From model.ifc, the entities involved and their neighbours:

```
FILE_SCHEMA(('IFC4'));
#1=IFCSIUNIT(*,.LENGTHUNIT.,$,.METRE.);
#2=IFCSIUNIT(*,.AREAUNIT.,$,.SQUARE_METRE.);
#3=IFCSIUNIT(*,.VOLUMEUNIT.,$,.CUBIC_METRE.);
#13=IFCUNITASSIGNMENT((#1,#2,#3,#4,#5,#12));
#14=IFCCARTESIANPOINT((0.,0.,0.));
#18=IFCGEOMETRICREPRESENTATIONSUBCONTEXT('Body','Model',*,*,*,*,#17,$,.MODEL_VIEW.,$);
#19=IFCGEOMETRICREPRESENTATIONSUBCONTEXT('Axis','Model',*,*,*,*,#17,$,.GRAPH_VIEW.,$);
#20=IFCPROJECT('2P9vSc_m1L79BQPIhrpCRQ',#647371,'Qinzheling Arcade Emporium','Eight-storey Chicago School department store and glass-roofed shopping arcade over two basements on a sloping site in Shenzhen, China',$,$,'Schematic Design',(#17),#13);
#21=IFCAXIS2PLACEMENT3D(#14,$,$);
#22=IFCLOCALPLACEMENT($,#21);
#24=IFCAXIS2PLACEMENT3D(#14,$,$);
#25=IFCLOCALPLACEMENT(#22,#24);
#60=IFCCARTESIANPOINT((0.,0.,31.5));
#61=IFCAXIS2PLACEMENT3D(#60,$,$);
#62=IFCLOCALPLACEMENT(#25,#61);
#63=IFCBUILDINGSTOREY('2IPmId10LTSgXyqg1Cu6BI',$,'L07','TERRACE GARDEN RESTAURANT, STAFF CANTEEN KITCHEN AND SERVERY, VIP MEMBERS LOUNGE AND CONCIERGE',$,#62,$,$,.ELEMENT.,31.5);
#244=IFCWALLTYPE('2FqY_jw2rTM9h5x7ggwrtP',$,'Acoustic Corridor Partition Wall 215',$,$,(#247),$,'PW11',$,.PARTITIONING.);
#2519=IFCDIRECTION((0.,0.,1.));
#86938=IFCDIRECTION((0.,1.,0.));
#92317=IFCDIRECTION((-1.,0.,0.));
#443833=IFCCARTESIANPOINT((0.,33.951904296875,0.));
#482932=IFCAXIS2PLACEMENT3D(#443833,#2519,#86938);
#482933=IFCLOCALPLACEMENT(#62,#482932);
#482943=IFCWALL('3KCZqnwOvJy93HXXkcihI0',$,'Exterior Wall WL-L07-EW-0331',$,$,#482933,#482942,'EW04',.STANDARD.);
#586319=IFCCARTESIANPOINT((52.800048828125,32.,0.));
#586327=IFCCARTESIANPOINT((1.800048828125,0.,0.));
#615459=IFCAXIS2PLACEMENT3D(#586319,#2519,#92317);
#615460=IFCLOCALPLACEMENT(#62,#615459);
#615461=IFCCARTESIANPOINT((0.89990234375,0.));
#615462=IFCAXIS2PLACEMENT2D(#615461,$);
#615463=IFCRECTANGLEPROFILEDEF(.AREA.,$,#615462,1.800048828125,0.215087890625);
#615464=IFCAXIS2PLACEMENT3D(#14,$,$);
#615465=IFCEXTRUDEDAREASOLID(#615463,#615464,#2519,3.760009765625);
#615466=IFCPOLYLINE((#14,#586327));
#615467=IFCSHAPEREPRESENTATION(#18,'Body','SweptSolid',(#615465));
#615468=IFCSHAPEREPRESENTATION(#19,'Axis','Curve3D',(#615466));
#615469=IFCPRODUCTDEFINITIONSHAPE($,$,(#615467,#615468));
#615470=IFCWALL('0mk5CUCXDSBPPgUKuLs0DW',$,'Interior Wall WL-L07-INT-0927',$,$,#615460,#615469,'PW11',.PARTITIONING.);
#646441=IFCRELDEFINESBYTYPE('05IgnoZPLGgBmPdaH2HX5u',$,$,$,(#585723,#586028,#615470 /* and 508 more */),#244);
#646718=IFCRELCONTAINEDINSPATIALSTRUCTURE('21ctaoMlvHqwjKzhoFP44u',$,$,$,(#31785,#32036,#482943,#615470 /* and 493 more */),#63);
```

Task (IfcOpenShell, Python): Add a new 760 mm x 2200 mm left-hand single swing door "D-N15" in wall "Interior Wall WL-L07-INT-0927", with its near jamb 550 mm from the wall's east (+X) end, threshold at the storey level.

```python
import numpy as np
import ifcopenshell
import ifcopenshell.api.feature
import ifcopenshell.api.geometry
import ifcopenshell.api.root
import ifcopenshell.api.spatial
import ifcopenshell.geom
import ifcopenshell.util.element
import ifcopenshell.util.placement
import ifcopenshell.util.representation
import ifcopenshell.util.shape
import ifcopenshell.util.unit

model = ifcopenshell.open("model.ifc")
unit_scale = ifcopenshell.util.unit.calculate_unit_scale(model)
settings = ifcopenshell.geom.settings()


def volume(element):
    """Net volume in cubic metres, openings subtracted."""
    shape = ifcopenshell.geom.create_shape(settings, element)
    return ifcopenshell.util.shape.get_volume(shape.geometry)


wall = model.by_guid("0mk5CUCXDSBPPgUKuLs0DW")
storey = ifcopenshell.util.element.get_container(wall, ifc_class="IfcBuildingStorey")
context = ifcopenshell.util.representation.get_context(model, "Model", "Body", "MODEL_VIEW")
before = volume(wall)

width, height, from_end, sill = 0.76, 2.2, 0.55, 0.0  # metres

# The wall runs along its own X axis, and the end named is its -X end.
wall_shape = ifcopenshell.geom.create_shape(settings, wall)
x, y, z = ifcopenshell.util.shape.get_vertices(wall_shape.geometry).T
start = x.min() + from_end
face, thickness = float(y.min()), float(y.max() - y.min())
wall_matrix = ifcopenshell.util.placement.get_local_placement(wall.ObjectPlacement)
level = ifcopenshell.util.placement.get_local_placement(storey.ObjectPlacement)[2, 3]


def in_wall(x, y):
    """Placement at x, y metres in the wall's axes, at sill height."""
    matrix = wall_matrix.copy()
    matrix[:, 3] = wall_matrix @ np.array([x / unit_scale, y / unit_scale, 0.0, 1.0])
    matrix[2, 3] = level + sill / unit_scale
    return matrix


# Opening: a box that overshoots both wall faces by 50 mm.
opening = ifcopenshell.api.root.create_entity(model, ifc_class="IfcOpeningElement", predefined_type="OPENING")
box = ifcopenshell.api.geometry.add_wall_representation(
    model, context=context, length=width, height=height, thickness=thickness + 0.1
)
ifcopenshell.api.geometry.assign_representation(model, product=opening, representation=box)
ifcopenshell.api.geometry.edit_object_placement(model, product=opening, matrix=in_wall(start, face - 0.05), is_si=False)
ifcopenshell.api.feature.add_feature(model, feature=opening, element=wall)

door = ifcopenshell.api.root.create_entity(model, ifc_class="IfcDoor", name="D-N15", predefined_type="DOOR")
door.OverallWidth, door.OverallHeight = width / unit_scale, height / unit_scale
door.OperationType = "SINGLE_SWING_LEFT"
body = ifcopenshell.api.geometry.add_door_representation(
    model,
    context=context,
    overall_width=door.OverallWidth,
    overall_height=door.OverallHeight,
    operation_type="SINGLE_SWING_LEFT",
    lining_properties={"LiningDepth": thickness / unit_scale, "ThresholdDepth": thickness / unit_scale},
)
ifcopenshell.api.geometry.assign_representation(model, product=door, representation=body)
ifcopenshell.api.spatial.assign_container(model, products=[door], relating_structure=storey)
ifcopenshell.api.feature.add_filling(model, opening=opening, element=door)

# The lining spans the wall, so the door starts at the wall face.
ifcopenshell.api.geometry.edit_object_placement(model, product=door, matrix=in_wall(start, face), is_si=False)

after = volume(wall)

print(f"wall volume {before:.3f} -> {after:.3f} m3")

model.write("model_rev.ifc")
```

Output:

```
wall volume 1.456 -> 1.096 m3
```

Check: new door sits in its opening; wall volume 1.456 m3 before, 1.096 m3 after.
